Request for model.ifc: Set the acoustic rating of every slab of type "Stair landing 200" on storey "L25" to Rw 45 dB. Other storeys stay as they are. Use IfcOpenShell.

First a look at what the model holds.

```python
import ifcopenshell
import ifcopenshell.util.element

model = ifcopenshell.open("model.ifc")
print(model.schema)
storey = next(s for s in model.by_type("IfcBuildingStorey") if s.Name == "L25")
slabs = [e for e in ifcopenshell.util.element.get_decomposition(storey) if e.is_a("IfcSlab")]
seen = {}
for e in slabs:
    element_type = ifcopenshell.util.element.get_type(e)
    key = (element_type.Name if element_type != e and element_type else None, ifcopenshell.util.element.get_pset(e, "Pset_SlabCommon", "AcousticRating"))
    seen[key] = seen.get(key, 0) + 1
for (name, value), count in sorted(seen.items(), key=str):
    print(count, "x", name, "|", value)
```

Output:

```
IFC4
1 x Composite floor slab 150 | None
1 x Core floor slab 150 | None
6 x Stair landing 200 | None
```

```python
import ifcopenshell
import ifcopenshell.api.pset
import ifcopenshell.util.element

model = ifcopenshell.open("model.ifc")

storey = next(s for s in model.by_type("IfcBuildingStorey") if s.Name == "L25")
slabs = [e for e in ifcopenshell.util.element.get_decomposition(storey) if e.is_a("IfcSlab")]

count = 0
for e in slabs:
    element_type = ifcopenshell.util.element.get_type(e)
    if element_type in (None, e) or element_type.Name != "Stair landing 200":
        continue
    found = ifcopenshell.util.element.get_pset(e, "Pset_SlabCommon", should_inherit=False)
    if found:
        pset = model.by_id(found["id"])
        if len(ifcopenshell.util.element.get_elements_by_pset(pset)) > 1:
            pset = ifcopenshell.api.pset.unshare_pset(model, products=[e], pset=pset)[0]
    else:
        pset = ifcopenshell.api.pset.add_pset(model, product=e, name="Pset_SlabCommon")
    ifcopenshell.api.pset.edit_pset(model, pset=pset, properties={"AcousticRating": "Rw 45 dB"})
    count += 1

print(count, "slabs updated")

model.write("model-out.ifc")
```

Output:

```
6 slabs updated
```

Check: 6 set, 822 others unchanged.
